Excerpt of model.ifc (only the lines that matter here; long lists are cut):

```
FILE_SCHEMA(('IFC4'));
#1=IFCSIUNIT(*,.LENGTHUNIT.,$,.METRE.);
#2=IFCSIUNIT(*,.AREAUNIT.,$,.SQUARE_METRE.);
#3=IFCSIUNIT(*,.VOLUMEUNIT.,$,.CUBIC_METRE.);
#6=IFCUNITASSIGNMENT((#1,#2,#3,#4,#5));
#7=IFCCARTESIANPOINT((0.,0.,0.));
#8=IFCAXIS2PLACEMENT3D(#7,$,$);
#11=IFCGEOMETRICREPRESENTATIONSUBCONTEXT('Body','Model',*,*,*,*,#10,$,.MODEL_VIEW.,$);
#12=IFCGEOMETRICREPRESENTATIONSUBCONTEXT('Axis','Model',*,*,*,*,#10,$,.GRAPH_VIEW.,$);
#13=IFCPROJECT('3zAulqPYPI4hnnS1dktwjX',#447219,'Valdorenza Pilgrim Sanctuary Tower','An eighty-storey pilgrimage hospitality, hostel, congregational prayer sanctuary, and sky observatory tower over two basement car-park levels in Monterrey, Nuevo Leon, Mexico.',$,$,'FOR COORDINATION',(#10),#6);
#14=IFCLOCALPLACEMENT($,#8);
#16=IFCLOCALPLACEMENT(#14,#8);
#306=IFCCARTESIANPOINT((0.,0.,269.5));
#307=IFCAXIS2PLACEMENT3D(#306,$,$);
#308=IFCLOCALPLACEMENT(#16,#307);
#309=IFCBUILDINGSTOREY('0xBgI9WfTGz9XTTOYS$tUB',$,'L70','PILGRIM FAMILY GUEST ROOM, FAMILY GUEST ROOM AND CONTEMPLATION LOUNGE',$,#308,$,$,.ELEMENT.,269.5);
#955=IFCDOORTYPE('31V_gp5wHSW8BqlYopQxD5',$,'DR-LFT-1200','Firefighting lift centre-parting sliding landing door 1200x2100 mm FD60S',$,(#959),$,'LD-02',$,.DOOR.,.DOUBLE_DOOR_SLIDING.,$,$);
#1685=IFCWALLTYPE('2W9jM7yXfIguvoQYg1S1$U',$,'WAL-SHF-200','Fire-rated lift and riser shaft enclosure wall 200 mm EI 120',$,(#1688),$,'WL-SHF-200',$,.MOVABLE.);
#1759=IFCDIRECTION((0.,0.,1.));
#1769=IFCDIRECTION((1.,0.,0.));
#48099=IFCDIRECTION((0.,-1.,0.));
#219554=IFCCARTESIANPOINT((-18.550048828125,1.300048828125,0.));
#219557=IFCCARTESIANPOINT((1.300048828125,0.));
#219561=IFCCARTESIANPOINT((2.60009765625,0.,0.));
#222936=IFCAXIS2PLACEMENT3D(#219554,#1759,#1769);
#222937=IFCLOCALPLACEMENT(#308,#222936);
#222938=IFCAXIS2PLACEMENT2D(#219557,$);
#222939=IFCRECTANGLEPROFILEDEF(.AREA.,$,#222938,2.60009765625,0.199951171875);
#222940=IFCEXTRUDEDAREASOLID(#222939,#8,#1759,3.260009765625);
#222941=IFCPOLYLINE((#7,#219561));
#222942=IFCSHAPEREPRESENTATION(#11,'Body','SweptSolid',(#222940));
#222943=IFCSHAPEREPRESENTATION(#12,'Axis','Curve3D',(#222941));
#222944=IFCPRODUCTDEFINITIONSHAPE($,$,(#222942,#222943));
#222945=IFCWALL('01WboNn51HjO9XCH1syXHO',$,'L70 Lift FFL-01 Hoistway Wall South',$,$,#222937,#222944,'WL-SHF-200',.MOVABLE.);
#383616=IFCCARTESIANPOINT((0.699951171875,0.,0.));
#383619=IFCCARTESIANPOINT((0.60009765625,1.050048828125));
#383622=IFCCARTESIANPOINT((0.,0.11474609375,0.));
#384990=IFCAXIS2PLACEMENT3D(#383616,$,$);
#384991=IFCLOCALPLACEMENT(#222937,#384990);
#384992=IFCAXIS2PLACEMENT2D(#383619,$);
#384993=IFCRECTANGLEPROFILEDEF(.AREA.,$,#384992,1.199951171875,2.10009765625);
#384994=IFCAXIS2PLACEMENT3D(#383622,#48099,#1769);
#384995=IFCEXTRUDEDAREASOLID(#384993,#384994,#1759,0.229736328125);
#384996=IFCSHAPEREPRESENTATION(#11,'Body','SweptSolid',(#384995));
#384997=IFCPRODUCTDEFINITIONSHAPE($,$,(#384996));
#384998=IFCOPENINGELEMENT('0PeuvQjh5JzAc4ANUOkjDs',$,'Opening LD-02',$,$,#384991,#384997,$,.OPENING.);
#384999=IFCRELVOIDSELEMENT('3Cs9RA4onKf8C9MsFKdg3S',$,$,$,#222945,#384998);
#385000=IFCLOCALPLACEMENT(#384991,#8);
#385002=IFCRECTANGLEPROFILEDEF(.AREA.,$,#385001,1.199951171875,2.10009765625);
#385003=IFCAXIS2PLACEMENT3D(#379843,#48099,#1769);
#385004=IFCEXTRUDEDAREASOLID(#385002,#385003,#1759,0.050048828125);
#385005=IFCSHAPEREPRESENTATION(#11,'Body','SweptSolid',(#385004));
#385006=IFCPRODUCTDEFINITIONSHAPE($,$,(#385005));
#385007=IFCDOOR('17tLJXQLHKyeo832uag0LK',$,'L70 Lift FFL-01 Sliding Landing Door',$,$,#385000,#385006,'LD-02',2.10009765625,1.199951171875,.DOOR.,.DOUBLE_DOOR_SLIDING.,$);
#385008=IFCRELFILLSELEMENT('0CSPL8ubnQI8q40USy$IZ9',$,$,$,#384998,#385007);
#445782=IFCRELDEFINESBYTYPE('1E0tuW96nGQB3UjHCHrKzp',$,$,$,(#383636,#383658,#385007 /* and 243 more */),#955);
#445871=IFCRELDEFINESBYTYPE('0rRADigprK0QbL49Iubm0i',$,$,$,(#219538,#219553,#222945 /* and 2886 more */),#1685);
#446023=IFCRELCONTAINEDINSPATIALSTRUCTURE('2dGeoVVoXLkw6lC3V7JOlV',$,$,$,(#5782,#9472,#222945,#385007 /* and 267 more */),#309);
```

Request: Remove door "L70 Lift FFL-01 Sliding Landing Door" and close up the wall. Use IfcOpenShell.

```python
import ifcopenshell
import ifcopenshell.api.feature
import ifcopenshell.api.root
import ifcopenshell.geom
import ifcopenshell.util.shape

model = ifcopenshell.open("model.ifc")
settings = ifcopenshell.geom.settings()


def volume(element):
    """Net volume in cubic metres, openings subtracted."""
    shape = ifcopenshell.geom.create_shape(settings, element)
    return ifcopenshell.util.shape.get_volume(shape.geometry)


door = model.by_id(385007)
opening = door.FillsVoids[0].RelatingOpeningElement
wall = opening.VoidsElements[0].RelatingBuildingElement
before = volume(wall)

ifcopenshell.api.root.remove_product(model, product=door)
ifcopenshell.api.feature.remove_feature(model, feature=opening)

after = volume(wall)

print(f"wall volume {before:.3f} -> {after:.3f} m3")

model.write("model-out.ifc")
```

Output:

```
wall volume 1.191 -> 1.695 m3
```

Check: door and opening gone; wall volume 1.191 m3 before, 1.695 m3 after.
